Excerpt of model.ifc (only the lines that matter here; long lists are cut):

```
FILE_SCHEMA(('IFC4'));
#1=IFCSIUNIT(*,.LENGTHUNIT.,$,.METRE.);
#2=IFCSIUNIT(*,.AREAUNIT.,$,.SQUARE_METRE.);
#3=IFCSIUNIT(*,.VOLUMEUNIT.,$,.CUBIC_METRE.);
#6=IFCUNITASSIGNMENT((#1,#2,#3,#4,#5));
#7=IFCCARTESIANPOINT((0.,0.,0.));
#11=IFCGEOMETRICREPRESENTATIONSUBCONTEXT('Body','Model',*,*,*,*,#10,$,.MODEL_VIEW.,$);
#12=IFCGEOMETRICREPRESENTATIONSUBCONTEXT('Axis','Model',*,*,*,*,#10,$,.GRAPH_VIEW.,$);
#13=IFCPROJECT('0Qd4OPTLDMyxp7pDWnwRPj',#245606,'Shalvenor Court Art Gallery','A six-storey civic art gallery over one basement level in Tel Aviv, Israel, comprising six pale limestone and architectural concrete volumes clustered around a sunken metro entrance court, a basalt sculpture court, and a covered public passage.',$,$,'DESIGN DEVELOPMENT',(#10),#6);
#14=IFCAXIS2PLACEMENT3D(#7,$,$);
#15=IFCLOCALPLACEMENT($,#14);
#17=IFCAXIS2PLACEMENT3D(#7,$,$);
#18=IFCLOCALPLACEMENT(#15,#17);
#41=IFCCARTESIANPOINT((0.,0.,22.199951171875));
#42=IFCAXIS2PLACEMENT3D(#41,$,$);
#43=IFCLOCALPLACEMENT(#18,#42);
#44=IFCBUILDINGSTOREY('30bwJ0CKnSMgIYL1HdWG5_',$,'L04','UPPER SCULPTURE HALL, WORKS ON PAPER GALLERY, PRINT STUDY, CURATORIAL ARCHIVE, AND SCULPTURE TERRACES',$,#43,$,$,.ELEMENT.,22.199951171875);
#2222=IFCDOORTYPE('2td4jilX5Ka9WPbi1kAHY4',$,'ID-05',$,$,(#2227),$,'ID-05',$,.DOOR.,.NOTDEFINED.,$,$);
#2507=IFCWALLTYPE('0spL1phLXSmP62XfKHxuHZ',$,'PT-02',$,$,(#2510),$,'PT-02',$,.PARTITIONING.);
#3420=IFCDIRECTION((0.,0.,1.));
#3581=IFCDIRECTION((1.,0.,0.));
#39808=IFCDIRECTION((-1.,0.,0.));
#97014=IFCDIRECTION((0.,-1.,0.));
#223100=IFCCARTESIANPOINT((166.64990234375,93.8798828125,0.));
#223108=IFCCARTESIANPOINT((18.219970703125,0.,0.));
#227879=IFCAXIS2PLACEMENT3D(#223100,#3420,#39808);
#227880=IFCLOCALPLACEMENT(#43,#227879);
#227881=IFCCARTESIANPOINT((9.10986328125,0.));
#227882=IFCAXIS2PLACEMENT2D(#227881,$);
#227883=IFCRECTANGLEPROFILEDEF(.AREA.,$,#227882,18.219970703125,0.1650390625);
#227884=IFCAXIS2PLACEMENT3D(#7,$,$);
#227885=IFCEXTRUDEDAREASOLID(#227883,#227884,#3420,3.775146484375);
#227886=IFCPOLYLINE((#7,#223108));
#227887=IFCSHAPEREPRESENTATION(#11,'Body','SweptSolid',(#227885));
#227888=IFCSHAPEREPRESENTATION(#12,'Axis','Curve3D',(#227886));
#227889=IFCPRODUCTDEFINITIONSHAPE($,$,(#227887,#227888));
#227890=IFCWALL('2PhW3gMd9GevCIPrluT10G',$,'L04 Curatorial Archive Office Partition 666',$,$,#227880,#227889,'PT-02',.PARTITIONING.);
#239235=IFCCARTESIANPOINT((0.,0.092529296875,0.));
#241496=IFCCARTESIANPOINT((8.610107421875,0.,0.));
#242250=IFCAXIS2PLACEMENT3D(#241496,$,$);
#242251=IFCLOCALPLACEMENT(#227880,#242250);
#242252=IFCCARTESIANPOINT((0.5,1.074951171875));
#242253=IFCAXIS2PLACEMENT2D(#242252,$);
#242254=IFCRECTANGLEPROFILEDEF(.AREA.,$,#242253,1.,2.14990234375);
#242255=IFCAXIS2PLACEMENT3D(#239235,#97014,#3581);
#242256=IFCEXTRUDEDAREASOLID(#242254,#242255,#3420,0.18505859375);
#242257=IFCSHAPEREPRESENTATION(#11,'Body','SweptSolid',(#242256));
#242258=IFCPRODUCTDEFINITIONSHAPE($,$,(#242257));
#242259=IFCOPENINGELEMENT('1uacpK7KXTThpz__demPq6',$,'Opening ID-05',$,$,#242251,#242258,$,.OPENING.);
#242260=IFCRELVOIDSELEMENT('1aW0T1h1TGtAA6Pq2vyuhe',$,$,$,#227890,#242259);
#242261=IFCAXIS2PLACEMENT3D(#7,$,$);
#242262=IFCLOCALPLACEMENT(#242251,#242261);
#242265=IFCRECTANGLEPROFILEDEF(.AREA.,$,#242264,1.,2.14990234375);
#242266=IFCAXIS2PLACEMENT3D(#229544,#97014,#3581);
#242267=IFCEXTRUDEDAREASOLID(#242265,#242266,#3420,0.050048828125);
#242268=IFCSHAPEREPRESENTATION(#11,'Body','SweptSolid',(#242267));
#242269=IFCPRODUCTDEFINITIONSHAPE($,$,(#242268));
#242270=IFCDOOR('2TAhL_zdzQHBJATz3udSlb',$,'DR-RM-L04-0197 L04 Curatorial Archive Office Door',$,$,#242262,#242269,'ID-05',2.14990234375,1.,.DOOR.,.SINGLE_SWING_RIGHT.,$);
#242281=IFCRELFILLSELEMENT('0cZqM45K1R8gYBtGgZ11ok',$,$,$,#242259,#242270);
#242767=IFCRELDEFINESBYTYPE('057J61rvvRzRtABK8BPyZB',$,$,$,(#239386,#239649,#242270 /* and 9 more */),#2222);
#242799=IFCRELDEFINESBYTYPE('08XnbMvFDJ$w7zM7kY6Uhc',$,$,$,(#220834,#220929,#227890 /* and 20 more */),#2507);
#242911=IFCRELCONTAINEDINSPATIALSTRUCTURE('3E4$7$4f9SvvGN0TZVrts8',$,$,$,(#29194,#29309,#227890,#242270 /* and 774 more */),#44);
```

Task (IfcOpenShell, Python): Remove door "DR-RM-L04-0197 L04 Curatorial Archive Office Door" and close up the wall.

```python
import ifcopenshell
import ifcopenshell.api.feature
import ifcopenshell.api.root
import ifcopenshell.geom
import ifcopenshell.util.shape

model = ifcopenshell.open("model.ifc")
settings = ifcopenshell.geom.settings()


def volume(element):
    """Net volume in cubic metres, openings subtracted."""
    shape = ifcopenshell.geom.create_shape(settings, element)
    return ifcopenshell.util.shape.get_volume(shape.geometry)


door = model.by_guid("2TAhL_zdzQHBJATz3udSlb")
opening = door.FillsVoids[0].RelatingOpeningElement
wall = opening.VoidsElements[0].RelatingBuildingElement
before = volume(wall)

ifcopenshell.api.root.remove_product(model, product=door)
ifcopenshell.api.feature.remove_feature(model, feature=opening)

after = volume(wall)

print(f"wall volume {before:.3f} -> {after:.3f} m3")

model.write("model-out.ifc")
```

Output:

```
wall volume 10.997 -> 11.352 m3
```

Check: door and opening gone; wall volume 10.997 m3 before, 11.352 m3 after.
